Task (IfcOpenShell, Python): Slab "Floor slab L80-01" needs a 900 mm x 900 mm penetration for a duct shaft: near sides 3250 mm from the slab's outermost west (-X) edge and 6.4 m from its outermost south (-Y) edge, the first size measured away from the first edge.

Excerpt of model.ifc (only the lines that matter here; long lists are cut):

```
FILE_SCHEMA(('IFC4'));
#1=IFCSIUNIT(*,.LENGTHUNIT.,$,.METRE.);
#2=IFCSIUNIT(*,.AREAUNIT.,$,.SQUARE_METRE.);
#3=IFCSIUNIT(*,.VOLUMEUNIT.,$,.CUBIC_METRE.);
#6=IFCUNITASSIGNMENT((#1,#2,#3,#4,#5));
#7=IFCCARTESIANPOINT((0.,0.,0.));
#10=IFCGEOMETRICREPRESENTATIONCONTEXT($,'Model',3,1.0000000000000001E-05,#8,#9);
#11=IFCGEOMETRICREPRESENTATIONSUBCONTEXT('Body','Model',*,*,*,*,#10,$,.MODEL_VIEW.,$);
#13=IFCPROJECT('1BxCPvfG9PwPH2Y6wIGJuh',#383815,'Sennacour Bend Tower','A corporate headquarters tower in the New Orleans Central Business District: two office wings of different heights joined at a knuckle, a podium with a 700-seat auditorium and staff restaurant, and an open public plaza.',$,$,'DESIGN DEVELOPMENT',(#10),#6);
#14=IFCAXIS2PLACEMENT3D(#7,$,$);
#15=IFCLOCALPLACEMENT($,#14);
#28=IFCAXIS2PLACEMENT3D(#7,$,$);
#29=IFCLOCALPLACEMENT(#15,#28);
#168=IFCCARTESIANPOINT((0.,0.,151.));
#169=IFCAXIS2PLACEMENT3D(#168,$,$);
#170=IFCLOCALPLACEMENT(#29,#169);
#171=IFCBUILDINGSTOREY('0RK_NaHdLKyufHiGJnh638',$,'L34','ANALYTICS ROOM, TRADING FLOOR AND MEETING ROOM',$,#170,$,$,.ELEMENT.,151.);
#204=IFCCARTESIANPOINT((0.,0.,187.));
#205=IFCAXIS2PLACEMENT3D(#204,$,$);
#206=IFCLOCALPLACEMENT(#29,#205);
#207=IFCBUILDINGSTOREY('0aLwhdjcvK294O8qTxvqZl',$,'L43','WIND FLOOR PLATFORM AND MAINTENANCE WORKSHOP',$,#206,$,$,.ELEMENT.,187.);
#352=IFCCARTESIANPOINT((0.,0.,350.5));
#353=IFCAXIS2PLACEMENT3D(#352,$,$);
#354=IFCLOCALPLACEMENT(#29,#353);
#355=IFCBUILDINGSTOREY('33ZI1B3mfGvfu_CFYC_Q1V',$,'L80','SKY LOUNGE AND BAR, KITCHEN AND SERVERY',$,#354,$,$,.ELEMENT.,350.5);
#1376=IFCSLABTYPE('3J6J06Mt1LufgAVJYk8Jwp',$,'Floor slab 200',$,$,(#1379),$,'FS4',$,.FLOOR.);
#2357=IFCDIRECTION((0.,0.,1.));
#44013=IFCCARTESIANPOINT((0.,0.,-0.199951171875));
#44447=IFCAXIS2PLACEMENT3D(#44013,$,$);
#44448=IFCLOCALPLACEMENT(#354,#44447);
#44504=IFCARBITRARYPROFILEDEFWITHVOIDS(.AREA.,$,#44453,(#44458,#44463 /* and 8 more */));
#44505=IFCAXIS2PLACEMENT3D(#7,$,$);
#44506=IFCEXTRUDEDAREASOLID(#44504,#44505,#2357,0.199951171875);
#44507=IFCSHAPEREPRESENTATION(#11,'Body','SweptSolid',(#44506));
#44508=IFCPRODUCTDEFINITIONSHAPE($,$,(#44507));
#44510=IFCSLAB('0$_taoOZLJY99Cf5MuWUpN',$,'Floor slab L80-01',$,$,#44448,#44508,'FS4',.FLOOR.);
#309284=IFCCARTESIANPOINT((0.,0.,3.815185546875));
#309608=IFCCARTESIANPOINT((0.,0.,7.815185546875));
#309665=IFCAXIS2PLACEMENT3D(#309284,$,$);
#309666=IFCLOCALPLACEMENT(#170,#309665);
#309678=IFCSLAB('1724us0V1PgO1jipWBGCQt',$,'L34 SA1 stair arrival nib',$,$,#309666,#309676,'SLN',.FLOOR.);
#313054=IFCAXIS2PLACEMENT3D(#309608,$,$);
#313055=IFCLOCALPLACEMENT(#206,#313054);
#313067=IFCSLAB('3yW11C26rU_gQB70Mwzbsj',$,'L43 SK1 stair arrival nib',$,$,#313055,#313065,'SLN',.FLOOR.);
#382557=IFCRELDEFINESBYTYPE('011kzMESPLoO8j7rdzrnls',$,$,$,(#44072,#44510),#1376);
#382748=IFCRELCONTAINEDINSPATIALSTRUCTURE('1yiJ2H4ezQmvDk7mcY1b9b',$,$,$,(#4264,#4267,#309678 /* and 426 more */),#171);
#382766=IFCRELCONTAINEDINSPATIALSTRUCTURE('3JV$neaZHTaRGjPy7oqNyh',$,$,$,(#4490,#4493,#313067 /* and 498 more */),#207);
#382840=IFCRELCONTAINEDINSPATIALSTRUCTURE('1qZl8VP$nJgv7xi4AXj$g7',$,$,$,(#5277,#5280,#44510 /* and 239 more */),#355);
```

```python
import numpy as np
import ifcopenshell
import ifcopenshell.api.feature
import ifcopenshell.api.geometry
import ifcopenshell.api.root
import ifcopenshell.geom
import ifcopenshell.util.placement
import ifcopenshell.util.representation
import ifcopenshell.util.shape
import ifcopenshell.util.unit

model = ifcopenshell.open("model.ifc")
unit_scale = ifcopenshell.util.unit.calculate_unit_scale(model)
settings = ifcopenshell.geom.settings()


def volume(element):
    """Net volume in cubic metres, openings subtracted."""
    shape = ifcopenshell.geom.create_shape(settings, element)
    return ifcopenshell.util.shape.get_volume(shape.geometry)


slab = model.by_guid("0$_taoOZLJY99Cf5MuWUpN")
before = volume(slab)

# Extent in the slab's own axes, in metres. The edges named are its -X and -Y sides.
slab_shape = ifcopenshell.geom.create_shape(settings, slab)
vertices = ifcopenshell.util.shape.get_vertices(slab_shape.geometry)
x_min, y_min, bottom = vertices.min(axis=0)
top = vertices[:, 2].max()

opening = ifcopenshell.api.root.create_entity(model, ifc_class="IfcOpeningElement", name="Duct shaft opening", predefined_type="OPENING")
context = ifcopenshell.util.representation.get_context(model, "Model", "Body", "MODEL_VIEW")
width, depth = 0.9, 0.9
outline = [(0.0, 0.0), (width, 0.0), (width, depth), (0.0, depth), (0.0, 0.0)]
# Overshoot both faces by 50 mm so the cut is clean.
shape = ifcopenshell.api.geometry.add_slab_representation(
    model, context=context, depth=top - bottom + 0.1, polyline=outline
)
ifcopenshell.api.geometry.assign_representation(model, product=opening, representation=shape)

matrix = ifcopenshell.util.placement.get_local_placement(slab.ObjectPlacement)
matrix[:, 3] = matrix @ np.append(np.array([x_min + 3.25, y_min + 6.4, bottom - 0.05]) / unit_scale, 1.0)
ifcopenshell.api.geometry.edit_object_placement(model, product=opening, matrix=matrix, is_si=False)
ifcopenshell.api.feature.add_feature(model, feature=opening, element=slab)

after = volume(slab)

print(f"slab volume {before:.3f} -> {after:.3f} m3")

model.write("model_updated.ifc")
```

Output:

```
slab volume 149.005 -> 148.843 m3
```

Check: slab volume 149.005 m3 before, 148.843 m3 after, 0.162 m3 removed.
